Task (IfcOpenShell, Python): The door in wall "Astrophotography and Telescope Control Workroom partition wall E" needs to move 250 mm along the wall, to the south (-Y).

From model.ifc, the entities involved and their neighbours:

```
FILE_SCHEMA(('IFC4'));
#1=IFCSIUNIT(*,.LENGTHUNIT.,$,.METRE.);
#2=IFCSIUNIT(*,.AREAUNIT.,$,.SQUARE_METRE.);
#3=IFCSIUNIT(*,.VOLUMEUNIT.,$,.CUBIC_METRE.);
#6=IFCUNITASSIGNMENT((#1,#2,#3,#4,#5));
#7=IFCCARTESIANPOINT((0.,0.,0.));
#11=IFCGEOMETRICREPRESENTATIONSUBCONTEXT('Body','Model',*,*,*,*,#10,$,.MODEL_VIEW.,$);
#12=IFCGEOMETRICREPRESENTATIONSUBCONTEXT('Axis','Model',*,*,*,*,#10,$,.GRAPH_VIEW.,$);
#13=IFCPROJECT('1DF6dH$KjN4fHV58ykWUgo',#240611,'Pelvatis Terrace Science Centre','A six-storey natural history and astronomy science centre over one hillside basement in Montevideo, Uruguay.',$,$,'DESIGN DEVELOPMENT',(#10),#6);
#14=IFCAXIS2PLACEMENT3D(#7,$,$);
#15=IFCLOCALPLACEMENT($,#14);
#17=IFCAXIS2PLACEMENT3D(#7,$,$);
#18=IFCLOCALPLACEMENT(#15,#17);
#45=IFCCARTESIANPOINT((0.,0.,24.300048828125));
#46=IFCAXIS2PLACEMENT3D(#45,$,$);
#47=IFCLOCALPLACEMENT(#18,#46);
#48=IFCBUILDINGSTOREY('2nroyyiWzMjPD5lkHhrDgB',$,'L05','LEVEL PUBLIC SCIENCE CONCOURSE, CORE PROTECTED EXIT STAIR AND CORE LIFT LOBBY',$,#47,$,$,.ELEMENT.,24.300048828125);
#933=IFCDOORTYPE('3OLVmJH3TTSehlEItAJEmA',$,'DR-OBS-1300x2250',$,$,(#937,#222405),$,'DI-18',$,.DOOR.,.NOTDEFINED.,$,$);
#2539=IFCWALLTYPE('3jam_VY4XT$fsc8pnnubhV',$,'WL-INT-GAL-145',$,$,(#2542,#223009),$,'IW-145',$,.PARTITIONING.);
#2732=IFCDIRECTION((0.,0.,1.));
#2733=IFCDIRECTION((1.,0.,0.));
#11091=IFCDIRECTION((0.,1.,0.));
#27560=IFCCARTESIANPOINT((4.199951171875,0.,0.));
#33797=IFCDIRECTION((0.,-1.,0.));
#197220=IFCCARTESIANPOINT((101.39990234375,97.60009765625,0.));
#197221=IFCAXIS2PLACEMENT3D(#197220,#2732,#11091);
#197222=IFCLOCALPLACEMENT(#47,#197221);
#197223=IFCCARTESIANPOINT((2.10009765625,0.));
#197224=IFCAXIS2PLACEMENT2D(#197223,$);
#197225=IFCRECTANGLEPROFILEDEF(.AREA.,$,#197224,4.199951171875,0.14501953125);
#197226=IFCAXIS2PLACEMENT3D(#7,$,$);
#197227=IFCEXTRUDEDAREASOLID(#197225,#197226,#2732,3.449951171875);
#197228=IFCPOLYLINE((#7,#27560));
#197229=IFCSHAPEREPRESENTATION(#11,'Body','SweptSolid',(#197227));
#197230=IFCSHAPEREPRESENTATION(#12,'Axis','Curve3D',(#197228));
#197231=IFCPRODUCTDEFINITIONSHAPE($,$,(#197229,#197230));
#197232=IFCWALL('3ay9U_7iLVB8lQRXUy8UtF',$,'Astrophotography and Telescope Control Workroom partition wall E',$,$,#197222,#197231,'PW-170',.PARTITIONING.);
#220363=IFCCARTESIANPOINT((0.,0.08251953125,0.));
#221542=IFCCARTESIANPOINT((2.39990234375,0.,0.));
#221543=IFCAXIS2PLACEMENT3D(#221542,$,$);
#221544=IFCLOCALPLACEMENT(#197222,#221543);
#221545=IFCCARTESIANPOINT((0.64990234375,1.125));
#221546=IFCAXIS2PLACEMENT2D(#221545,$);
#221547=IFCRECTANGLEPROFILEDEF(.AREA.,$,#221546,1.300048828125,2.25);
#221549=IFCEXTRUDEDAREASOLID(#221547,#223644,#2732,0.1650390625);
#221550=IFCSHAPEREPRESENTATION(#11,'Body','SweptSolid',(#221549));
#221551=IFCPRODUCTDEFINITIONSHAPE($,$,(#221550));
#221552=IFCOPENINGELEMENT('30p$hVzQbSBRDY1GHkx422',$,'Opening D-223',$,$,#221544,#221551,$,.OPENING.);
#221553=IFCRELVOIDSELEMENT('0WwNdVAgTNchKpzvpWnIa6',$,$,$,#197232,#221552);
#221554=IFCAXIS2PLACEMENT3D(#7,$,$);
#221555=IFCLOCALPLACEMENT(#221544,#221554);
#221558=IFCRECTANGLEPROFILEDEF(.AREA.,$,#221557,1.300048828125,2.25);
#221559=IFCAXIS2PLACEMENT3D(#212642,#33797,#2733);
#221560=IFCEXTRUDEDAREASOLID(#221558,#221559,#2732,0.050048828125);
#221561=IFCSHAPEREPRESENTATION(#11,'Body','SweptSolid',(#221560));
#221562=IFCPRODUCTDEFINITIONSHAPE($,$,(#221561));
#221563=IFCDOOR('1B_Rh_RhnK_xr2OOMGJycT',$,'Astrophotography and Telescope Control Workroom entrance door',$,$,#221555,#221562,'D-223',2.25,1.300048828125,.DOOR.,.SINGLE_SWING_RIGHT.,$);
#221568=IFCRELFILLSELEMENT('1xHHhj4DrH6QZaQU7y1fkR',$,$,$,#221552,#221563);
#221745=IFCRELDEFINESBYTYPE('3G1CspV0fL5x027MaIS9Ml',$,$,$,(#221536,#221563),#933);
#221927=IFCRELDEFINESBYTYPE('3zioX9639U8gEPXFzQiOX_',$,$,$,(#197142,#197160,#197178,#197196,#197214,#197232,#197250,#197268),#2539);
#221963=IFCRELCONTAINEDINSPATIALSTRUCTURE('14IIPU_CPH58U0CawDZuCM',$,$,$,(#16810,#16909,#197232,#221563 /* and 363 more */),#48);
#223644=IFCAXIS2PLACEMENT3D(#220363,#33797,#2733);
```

```python
import ifcopenshell
import ifcopenshell.api.geometry
import ifcopenshell.util.placement
import ifcopenshell.util.unit

model = ifcopenshell.open("model.ifc")
unit_scale = ifcopenshell.util.unit.calculate_unit_scale(model)

door = model.by_guid("1B_Rh_RhnK_xr2OOMGJycT")
opening = door.FillsVoids[0].RelatingOpeningElement
wall = opening.VoidsElements[0].RelatingBuildingElement

wall_matrix = ifcopenshell.util.placement.get_local_placement(wall.ObjectPlacement)
shift = wall_matrix[:3, 0] * -0.25 / unit_scale
before = ifcopenshell.util.placement.get_local_placement(door.ObjectPlacement)[:3, 3].copy()

# The door is placed relative to its opening, so it follows when the opening moves.
matrix = ifcopenshell.util.placement.get_local_placement(opening.ObjectPlacement)
matrix[:3, 3] += shift
ifcopenshell.api.geometry.edit_object_placement(
    model, product=opening, matrix=matrix, is_si=False, should_transform_children=True
)

after = ifcopenshell.util.placement.get_local_placement(door.ObjectPlacement)[:3, 3]
print("door moved by", (after - before).round(3) + 0.0)

model.write("model-out.ifc")
```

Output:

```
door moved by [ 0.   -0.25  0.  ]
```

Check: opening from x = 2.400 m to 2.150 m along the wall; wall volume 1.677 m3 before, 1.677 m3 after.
